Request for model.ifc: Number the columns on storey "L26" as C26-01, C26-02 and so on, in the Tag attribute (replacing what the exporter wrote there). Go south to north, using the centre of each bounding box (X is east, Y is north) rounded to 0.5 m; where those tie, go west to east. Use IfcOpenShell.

First a look at what the model holds.

```python
import ifcopenshell
import ifcopenshell.util.element
import ifcopenshell.util.placement

model = ifcopenshell.open("model.ifc")
print(model.schema)
storey = next(s for s in model.by_type("IfcBuildingStorey") if s.Name == "L26")
columns = [e for e in ifcopenshell.util.element.get_decomposition(storey) if e.is_a("IfcColumn")]
for e in sorted(columns, key=lambda e: e.id()):
    origin = ifcopenshell.util.placement.get_local_placement(e.ObjectPlacement)[:3, 3]
    print(e.id(), e.Tag, e.Name, origin.round(2) + 0.0, sep=" | ")
```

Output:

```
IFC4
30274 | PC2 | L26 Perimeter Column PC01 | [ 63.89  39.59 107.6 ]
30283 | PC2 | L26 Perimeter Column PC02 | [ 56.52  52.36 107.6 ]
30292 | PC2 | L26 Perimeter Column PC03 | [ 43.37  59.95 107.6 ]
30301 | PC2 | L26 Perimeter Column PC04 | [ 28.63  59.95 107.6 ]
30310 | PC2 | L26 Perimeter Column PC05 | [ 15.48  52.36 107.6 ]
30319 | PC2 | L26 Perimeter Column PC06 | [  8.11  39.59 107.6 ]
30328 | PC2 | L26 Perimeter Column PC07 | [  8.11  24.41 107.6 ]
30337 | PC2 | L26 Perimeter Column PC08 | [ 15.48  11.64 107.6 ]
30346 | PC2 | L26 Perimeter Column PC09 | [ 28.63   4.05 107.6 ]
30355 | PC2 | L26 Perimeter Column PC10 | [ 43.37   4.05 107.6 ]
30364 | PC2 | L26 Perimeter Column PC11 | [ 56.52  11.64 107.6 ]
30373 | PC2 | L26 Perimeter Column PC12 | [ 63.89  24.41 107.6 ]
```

```python
import ifcopenshell
import ifcopenshell.geom
import ifcopenshell.util.element
import ifcopenshell.util.shape

model = ifcopenshell.open("model.ifc")
settings = ifcopenshell.geom.settings()
settings.set("use-world-coords", True)


def centre(element):
    shape = ifcopenshell.geom.create_shape(settings, element)
    return ifcopenshell.util.shape.get_bbox_centroid(shape.geometry)


storey = next(s for s in model.by_type("IfcBuildingStorey") if s.Name == "L26")
columns = [e for e in ifcopenshell.util.element.get_decomposition(storey) if e.is_a("IfcColumn")]

# Insertion points can sit at a corner or the storey origin, so sort by the geometry (in metres).
centres = {e: centre(e) for e in columns}
columns.sort(key=lambda e: (round(centres[e][1] / 0.5), centres[e][0]))

for i, e in enumerate(columns, start=1):
    number = f"C26-{i:02d}"
    e.Tag = number
    print(e.id(), number)

model.write("model_v2.ifc")
```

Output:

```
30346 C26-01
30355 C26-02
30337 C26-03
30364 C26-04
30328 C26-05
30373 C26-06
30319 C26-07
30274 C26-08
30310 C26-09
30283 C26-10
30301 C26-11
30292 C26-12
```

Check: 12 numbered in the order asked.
